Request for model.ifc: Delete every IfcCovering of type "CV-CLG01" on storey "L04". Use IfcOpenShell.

First a look at what the model holds.

```python
import ifcopenshell
import ifcopenshell.util.element

model = ifcopenshell.open("model.ifc")
print(model.schema)
storey = next(s for s in model.by_type("IfcBuildingStorey") if s.Name == "L04")
coverings = [e for e in ifcopenshell.util.element.get_decomposition(storey) if e.is_a("IfcCovering")]
seen = {}
for e in coverings:
    element_type = ifcopenshell.util.element.get_type(e)
    name = element_type.Name if element_type not in (None, e) else None
    seen[name] = seen.get(name, 0) + 1
for name, count in sorted(seen.items(), key=str):
    print(count, "x", name)
```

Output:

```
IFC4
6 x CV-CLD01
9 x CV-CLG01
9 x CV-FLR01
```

```python
import ifcopenshell
import ifcopenshell.api.root
import ifcopenshell.util.element

model = ifcopenshell.open("model.ifc")

storey = next(s for s in model.by_type("IfcBuildingStorey") if s.Name == "L04")
coverings = [e for e in ifcopenshell.util.element.get_decomposition(storey) if e.is_a("IfcCovering")]
targets = [e for e in coverings if (t := ifcopenshell.util.element.get_type(e)) not in (None, e) and t.Name == "CV-CLG01"]

for e in targets:
    ifcopenshell.api.root.remove_product(model, product=e)
print(len(targets), "removed")

model.write("model_edited.ifc")
```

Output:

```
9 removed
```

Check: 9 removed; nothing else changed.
